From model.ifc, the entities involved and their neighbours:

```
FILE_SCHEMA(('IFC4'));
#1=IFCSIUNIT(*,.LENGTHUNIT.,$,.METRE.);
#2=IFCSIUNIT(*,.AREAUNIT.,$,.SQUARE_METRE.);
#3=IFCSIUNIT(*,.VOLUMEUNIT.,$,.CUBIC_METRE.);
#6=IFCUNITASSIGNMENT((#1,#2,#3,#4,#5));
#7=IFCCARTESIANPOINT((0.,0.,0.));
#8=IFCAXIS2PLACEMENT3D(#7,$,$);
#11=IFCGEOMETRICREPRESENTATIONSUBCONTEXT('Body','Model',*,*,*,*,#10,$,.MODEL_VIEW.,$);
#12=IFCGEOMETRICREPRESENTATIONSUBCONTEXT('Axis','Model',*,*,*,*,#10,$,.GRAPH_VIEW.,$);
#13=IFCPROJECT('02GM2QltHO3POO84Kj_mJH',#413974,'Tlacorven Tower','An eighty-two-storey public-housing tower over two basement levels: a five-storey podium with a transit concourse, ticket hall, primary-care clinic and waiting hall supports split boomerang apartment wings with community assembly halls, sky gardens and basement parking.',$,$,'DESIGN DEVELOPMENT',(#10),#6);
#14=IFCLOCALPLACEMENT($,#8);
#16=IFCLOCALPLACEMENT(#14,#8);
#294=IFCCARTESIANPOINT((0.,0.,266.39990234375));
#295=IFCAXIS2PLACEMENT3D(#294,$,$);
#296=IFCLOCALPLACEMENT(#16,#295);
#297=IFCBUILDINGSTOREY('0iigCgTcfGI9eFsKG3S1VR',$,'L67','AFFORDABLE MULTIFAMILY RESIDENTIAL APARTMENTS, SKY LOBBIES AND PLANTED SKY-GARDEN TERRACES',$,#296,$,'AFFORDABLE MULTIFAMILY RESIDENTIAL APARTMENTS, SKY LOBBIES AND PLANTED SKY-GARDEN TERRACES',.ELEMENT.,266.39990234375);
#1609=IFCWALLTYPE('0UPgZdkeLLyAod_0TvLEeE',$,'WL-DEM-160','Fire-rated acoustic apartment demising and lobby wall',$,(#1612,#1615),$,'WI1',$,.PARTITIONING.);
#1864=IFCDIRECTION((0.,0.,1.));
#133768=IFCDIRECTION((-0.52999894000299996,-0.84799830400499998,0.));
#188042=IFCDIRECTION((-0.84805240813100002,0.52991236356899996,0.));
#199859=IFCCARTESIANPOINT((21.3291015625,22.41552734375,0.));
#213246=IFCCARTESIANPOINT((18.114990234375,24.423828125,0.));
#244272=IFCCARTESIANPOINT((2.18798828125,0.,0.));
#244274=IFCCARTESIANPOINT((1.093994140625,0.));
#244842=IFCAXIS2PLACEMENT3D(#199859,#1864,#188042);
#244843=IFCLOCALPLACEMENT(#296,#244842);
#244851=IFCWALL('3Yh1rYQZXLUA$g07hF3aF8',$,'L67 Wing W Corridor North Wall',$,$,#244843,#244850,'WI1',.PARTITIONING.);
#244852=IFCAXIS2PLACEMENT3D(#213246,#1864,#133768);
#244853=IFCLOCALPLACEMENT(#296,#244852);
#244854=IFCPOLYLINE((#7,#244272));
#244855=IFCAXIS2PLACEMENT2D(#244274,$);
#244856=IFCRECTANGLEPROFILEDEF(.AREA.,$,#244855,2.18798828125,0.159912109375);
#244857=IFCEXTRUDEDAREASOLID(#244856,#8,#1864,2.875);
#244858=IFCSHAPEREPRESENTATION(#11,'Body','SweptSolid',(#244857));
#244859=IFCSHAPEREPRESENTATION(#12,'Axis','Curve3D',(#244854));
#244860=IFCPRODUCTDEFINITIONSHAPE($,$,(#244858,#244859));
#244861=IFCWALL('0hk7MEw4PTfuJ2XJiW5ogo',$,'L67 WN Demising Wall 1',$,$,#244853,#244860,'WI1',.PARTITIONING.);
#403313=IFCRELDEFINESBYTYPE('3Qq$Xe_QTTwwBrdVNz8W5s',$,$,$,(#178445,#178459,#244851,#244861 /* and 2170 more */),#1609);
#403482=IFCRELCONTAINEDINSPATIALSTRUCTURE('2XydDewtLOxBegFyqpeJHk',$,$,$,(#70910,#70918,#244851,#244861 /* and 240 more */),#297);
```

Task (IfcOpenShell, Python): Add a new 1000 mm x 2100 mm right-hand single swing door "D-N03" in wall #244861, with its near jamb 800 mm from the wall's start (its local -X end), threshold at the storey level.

```python
import numpy as np
import ifcopenshell
import ifcopenshell.api.feature
import ifcopenshell.api.geometry
import ifcopenshell.api.root
import ifcopenshell.api.spatial
import ifcopenshell.geom
import ifcopenshell.util.element
import ifcopenshell.util.placement
import ifcopenshell.util.representation
import ifcopenshell.util.shape
import ifcopenshell.util.unit

model = ifcopenshell.open("model.ifc")
unit_scale = ifcopenshell.util.unit.calculate_unit_scale(model)
settings = ifcopenshell.geom.settings()


def volume(element):
    """Net volume in cubic metres, openings subtracted."""
    shape = ifcopenshell.geom.create_shape(settings, element)
    return ifcopenshell.util.shape.get_volume(shape.geometry)


wall = model.by_guid("0hk7MEw4PTfuJ2XJiW5ogo")
storey = ifcopenshell.util.element.get_container(wall, ifc_class="IfcBuildingStorey")
context = ifcopenshell.util.representation.get_context(model, "Model", "Body", "MODEL_VIEW")
before = volume(wall)

width, height, from_end, sill = 1, 2.1, 0.8, 0.0  # metres

# The wall runs along its own X axis, and the end named is its -X end.
wall_shape = ifcopenshell.geom.create_shape(settings, wall)
x, y, z = ifcopenshell.util.shape.get_vertices(wall_shape.geometry).T
start = x.min() + from_end
face, thickness = float(y.min()), float(y.max() - y.min())
wall_matrix = ifcopenshell.util.placement.get_local_placement(wall.ObjectPlacement)
level = ifcopenshell.util.placement.get_local_placement(storey.ObjectPlacement)[2, 3]


def in_wall(x, y):
    """Placement at x, y metres in the wall's axes, at sill height."""
    matrix = wall_matrix.copy()
    matrix[:, 3] = wall_matrix @ np.array([x / unit_scale, y / unit_scale, 0.0, 1.0])
    matrix[2, 3] = level + sill / unit_scale
    return matrix


# Opening: a box that overshoots both wall faces by 50 mm.
opening = ifcopenshell.api.root.create_entity(model, ifc_class="IfcOpeningElement", predefined_type="OPENING")
box = ifcopenshell.api.geometry.add_wall_representation(
    model, context=context, length=width, height=height, thickness=thickness + 0.1
)
ifcopenshell.api.geometry.assign_representation(model, product=opening, representation=box)
ifcopenshell.api.geometry.edit_object_placement(model, product=opening, matrix=in_wall(start, face - 0.05), is_si=False)
ifcopenshell.api.feature.add_feature(model, feature=opening, element=wall)

door = ifcopenshell.api.root.create_entity(model, ifc_class="IfcDoor", name="D-N03", predefined_type="DOOR")
door.OverallWidth, door.OverallHeight = width / unit_scale, height / unit_scale
door.OperationType = "SINGLE_SWING_RIGHT"
body = ifcopenshell.api.geometry.add_door_representation(
    model,
    context=context,
    overall_width=door.OverallWidth,
    overall_height=door.OverallHeight,
    operation_type="SINGLE_SWING_RIGHT",
    lining_properties={"LiningDepth": thickness / unit_scale, "ThresholdDepth": thickness / unit_scale},
)
ifcopenshell.api.geometry.assign_representation(model, product=door, representation=body)
ifcopenshell.api.spatial.assign_container(model, products=[door], relating_structure=storey)
ifcopenshell.api.feature.add_filling(model, opening=opening, element=door)

# The lining spans the wall, so the door starts at the wall face.
ifcopenshell.api.geometry.edit_object_placement(model, product=door, matrix=in_wall(start, face), is_si=False)

after = volume(wall)

print(f"wall volume {before:.3f} -> {after:.3f} m3")

model.write("model-out.ifc")
```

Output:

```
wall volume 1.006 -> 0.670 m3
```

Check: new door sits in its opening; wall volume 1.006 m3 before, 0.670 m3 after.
